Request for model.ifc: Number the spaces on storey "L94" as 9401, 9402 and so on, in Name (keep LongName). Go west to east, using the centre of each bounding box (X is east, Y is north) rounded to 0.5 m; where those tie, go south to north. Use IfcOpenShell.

First a look at what the model holds.

```python
import ifcopenshell
import ifcopenshell.util.element
import ifcopenshell.util.placement

model = ifcopenshell.open("model.ifc")
print(model.schema)
storey = next(s for s in model.by_type("IfcBuildingStorey") if s.Name == "L94")
spaces = [e for e in ifcopenshell.util.element.get_decomposition(storey) if e.is_a("IfcSpace")]
for e in sorted(spaces, key=lambda e: e.id()):
    origin = ifcopenshell.util.placement.get_local_placement(e.ObjectPlacement)[:3, 3]
    print(e.id(), e.Name, e.LongName, origin.round(2) + 0.0, sep=" | ")
```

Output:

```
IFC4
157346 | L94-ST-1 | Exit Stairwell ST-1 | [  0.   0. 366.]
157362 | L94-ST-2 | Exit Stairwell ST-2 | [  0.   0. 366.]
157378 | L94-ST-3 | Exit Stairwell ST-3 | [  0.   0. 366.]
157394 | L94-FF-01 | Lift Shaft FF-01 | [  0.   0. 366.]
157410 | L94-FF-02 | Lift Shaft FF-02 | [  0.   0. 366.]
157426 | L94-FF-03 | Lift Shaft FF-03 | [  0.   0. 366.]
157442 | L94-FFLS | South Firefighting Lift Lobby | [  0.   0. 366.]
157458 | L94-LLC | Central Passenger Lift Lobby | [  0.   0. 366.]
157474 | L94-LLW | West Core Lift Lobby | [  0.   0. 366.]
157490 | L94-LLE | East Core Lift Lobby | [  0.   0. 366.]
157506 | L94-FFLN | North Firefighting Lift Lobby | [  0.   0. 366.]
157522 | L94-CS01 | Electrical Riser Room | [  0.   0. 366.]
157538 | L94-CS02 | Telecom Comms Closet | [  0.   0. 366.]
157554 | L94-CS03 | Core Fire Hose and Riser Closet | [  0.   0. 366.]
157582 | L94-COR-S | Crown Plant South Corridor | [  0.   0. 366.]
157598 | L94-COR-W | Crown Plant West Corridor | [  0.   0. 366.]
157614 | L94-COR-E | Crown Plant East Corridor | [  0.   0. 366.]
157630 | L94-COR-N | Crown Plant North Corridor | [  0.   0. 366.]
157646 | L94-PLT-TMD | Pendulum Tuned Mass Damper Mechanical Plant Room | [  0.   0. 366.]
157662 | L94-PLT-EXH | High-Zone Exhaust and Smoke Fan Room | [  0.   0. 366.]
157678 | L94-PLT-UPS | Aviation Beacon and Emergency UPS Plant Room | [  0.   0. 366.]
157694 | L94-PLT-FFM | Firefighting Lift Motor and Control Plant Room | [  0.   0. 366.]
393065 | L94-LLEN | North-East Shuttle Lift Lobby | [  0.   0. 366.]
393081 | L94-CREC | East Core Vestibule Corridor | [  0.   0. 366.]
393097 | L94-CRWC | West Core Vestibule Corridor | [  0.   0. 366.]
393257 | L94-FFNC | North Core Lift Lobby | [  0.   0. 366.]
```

```python
import ifcopenshell
import ifcopenshell.geom
import ifcopenshell.util.element
import ifcopenshell.util.shape

model = ifcopenshell.open("model.ifc")
settings = ifcopenshell.geom.settings()
settings.set("use-world-coords", True)


def centre(element):
    shape = ifcopenshell.geom.create_shape(settings, element)
    return ifcopenshell.util.shape.get_bbox_centroid(shape.geometry)


storey = next(s for s in model.by_type("IfcBuildingStorey") if s.Name == "L94")
spaces = [e for e in ifcopenshell.util.element.get_decomposition(storey) if e.is_a("IfcSpace")]

# Insertion points can sit at a corner or the storey origin, so sort by the geometry (in metres).
centres = {e: centre(e) for e in spaces}
spaces.sort(key=lambda e: (round(centres[e][0] / 0.5), centres[e][1]))

for i, e in enumerate(spaces, start=1):
    number = f"94{i:02d}"
    e.Name = number
    print(e.id(), number)

model.write("model-out.ifc")
```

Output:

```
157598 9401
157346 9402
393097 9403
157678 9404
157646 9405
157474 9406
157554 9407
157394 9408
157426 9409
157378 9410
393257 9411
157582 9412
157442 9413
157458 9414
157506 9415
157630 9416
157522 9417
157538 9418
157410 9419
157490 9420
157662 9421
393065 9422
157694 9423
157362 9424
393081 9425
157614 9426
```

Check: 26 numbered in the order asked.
